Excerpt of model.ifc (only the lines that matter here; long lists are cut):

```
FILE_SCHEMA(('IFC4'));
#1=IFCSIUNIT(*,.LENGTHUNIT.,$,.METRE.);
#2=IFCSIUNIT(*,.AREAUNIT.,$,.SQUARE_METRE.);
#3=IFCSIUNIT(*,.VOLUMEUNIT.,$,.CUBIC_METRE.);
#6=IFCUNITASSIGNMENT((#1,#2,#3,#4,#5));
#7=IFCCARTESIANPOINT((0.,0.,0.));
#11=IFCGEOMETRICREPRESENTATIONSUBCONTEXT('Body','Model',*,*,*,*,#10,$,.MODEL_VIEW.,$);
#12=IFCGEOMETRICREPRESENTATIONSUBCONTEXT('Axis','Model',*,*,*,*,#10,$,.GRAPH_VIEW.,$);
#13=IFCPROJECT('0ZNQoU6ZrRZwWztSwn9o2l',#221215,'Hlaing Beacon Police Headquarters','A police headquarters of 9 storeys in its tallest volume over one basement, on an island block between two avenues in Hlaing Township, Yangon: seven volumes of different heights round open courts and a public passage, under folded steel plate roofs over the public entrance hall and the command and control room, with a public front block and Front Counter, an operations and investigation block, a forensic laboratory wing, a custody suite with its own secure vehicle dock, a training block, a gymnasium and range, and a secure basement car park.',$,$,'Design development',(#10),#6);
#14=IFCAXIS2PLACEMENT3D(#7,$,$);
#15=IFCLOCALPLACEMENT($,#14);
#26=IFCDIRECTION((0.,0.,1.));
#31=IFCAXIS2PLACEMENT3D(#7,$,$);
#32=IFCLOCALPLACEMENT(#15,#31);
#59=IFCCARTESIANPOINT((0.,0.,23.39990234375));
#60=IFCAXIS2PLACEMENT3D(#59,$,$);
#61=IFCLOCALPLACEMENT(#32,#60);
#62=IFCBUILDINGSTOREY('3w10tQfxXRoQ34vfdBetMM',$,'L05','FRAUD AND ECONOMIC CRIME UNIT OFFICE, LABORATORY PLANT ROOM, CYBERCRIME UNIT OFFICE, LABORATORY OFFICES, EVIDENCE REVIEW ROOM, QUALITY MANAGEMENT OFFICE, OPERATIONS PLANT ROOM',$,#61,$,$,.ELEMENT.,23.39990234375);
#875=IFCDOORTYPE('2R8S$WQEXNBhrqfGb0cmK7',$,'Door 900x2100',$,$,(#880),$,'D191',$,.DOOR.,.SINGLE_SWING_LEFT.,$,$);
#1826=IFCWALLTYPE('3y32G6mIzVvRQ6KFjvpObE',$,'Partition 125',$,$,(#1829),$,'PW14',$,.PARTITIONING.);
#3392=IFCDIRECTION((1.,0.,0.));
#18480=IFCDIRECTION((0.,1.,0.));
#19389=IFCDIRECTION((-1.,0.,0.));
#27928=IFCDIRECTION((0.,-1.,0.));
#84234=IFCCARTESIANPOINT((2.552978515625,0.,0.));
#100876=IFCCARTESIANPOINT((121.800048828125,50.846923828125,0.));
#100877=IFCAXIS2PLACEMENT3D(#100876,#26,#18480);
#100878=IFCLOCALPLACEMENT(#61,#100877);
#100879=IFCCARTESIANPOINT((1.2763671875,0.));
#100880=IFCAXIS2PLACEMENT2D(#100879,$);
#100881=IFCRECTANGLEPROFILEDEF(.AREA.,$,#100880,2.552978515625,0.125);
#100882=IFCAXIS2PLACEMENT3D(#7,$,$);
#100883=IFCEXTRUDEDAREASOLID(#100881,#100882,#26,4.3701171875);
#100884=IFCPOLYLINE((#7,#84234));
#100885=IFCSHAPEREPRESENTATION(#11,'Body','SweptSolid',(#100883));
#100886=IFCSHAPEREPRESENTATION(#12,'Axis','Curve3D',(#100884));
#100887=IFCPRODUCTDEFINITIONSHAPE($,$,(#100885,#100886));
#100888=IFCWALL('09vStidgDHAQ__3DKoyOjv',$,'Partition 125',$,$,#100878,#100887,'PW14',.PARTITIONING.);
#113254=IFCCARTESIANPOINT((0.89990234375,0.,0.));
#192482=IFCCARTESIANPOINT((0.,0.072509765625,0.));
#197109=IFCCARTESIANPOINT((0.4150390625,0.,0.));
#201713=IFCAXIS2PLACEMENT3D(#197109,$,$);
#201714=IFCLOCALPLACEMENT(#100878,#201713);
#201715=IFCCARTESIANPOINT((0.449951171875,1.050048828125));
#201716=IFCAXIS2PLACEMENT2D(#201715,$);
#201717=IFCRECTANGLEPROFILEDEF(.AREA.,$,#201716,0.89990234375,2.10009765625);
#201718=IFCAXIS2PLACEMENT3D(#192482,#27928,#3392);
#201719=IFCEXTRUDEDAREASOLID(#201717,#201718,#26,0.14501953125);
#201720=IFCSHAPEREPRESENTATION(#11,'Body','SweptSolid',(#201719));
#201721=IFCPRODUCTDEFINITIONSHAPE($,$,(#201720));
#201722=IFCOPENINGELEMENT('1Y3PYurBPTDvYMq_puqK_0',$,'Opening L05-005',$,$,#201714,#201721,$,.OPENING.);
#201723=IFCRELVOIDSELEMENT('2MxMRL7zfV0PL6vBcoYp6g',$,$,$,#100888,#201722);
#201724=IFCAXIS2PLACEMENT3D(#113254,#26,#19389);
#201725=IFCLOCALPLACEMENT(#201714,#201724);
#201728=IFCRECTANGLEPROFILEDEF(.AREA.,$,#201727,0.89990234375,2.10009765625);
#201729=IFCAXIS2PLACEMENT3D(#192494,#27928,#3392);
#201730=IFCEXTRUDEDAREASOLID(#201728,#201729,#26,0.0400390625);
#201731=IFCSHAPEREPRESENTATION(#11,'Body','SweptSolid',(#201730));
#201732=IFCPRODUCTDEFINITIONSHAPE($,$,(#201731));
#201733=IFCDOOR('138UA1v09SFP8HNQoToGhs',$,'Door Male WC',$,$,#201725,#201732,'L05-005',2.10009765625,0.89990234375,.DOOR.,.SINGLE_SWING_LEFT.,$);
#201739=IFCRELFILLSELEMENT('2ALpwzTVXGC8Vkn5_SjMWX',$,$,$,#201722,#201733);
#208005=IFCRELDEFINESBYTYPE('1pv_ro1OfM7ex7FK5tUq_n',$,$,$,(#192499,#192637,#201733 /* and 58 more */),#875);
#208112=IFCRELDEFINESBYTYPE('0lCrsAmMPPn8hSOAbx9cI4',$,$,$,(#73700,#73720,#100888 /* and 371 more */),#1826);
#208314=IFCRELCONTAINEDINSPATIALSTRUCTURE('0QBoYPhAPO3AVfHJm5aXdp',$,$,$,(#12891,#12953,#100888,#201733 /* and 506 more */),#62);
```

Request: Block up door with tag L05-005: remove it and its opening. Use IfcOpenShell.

```python
import ifcopenshell
import ifcopenshell.api.feature
import ifcopenshell.api.root
import ifcopenshell.geom
import ifcopenshell.util.shape

model = ifcopenshell.open("model.ifc")
settings = ifcopenshell.geom.settings()


def volume(element):
    """Net volume in cubic metres, openings subtracted."""
    shape = ifcopenshell.geom.create_shape(settings, element)
    return ifcopenshell.util.shape.get_volume(shape.geometry)


door = model.by_id(201733)
opening = door.FillsVoids[0].RelatingOpeningElement
wall = opening.VoidsElements[0].RelatingBuildingElement
before = volume(wall)

ifcopenshell.api.root.remove_product(model, product=door)
ifcopenshell.api.feature.remove_feature(model, feature=opening)

after = volume(wall)

print(f"wall volume {before:.3f} -> {after:.3f} m3")

model.write("model_rev.ifc")
```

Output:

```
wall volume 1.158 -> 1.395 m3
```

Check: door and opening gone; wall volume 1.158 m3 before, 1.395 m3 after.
